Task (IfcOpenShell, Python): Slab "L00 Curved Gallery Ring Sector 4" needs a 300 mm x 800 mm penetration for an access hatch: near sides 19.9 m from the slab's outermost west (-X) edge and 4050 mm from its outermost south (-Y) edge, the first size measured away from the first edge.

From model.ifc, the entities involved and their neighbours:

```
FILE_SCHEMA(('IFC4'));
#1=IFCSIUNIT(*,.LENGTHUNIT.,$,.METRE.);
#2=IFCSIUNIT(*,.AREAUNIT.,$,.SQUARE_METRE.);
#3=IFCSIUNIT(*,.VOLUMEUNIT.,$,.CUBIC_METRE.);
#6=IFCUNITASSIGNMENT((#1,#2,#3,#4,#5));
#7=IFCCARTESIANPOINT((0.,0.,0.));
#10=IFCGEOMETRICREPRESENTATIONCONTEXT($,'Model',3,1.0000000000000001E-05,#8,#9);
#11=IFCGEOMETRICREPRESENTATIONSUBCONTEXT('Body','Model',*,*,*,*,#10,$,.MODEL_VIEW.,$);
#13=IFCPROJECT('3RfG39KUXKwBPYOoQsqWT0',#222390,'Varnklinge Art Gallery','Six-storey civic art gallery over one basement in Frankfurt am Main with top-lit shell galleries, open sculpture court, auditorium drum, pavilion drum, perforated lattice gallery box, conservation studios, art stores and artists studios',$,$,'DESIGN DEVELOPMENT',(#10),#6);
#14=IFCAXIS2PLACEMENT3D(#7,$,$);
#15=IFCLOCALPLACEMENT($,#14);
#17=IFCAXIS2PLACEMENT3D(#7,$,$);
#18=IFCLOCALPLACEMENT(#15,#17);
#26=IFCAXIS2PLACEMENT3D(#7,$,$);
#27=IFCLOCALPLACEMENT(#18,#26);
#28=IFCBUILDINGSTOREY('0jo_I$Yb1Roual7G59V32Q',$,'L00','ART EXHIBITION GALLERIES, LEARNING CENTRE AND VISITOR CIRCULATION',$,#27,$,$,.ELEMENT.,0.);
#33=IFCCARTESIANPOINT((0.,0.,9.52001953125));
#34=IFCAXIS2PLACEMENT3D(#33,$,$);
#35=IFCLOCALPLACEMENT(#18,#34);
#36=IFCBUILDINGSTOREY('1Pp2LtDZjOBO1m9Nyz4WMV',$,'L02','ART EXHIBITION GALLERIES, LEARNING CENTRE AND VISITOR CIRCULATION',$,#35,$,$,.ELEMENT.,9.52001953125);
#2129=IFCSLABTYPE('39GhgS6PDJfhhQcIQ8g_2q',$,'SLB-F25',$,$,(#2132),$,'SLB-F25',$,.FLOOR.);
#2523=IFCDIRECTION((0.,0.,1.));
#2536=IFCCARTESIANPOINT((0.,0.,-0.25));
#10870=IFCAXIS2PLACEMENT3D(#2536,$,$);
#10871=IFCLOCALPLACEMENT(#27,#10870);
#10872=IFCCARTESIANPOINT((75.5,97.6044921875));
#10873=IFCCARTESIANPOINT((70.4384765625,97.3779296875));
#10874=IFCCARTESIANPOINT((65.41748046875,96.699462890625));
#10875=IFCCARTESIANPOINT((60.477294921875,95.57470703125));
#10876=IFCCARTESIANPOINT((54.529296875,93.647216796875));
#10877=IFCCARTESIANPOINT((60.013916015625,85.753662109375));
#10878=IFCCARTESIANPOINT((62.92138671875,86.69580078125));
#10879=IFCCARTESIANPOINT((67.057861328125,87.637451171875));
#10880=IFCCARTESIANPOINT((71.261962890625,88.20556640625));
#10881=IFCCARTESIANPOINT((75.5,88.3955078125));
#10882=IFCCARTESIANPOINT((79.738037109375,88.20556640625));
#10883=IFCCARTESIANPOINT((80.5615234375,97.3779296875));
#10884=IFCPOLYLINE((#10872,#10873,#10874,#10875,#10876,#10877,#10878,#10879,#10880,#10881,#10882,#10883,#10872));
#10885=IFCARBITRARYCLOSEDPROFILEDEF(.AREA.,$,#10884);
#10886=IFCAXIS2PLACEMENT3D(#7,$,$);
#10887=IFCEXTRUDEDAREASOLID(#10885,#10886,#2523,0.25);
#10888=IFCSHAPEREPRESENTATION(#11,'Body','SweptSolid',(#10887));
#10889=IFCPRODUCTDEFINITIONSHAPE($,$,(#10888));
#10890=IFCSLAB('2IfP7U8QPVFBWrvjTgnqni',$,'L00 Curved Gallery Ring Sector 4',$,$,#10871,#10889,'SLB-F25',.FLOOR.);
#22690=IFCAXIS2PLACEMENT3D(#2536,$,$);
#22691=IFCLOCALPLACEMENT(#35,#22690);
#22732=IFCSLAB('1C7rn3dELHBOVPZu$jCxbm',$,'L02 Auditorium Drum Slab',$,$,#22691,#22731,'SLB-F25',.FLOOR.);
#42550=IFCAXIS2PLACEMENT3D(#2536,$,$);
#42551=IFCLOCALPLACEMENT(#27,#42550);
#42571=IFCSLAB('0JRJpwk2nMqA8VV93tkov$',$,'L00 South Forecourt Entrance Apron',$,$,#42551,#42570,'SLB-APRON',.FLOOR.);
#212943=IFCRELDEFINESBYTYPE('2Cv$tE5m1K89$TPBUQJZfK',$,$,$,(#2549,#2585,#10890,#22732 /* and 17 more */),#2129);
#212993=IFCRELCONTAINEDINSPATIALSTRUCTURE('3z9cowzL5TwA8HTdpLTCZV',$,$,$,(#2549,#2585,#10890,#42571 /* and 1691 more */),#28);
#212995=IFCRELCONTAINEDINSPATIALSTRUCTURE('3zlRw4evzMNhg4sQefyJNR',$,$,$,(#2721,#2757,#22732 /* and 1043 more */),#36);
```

```python
import numpy as np
import ifcopenshell
import ifcopenshell.api.feature
import ifcopenshell.api.geometry
import ifcopenshell.api.root
import ifcopenshell.geom
import ifcopenshell.util.placement
import ifcopenshell.util.representation
import ifcopenshell.util.shape
import ifcopenshell.util.unit

model = ifcopenshell.open("model.ifc")
unit_scale = ifcopenshell.util.unit.calculate_unit_scale(model)
settings = ifcopenshell.geom.settings()


def volume(element):
    """Net volume in cubic metres, openings subtracted."""
    shape = ifcopenshell.geom.create_shape(settings, element)
    return ifcopenshell.util.shape.get_volume(shape.geometry)


slab = model.by_guid("2IfP7U8QPVFBWrvjTgnqni")
before = volume(slab)

# Extent in the slab's own axes, in metres. The edges named are its -X and -Y sides.
slab_shape = ifcopenshell.geom.create_shape(settings, slab)
vertices = ifcopenshell.util.shape.get_vertices(slab_shape.geometry)
x_min, y_min, bottom = vertices.min(axis=0)
top = vertices[:, 2].max()

opening = ifcopenshell.api.root.create_entity(model, ifc_class="IfcOpeningElement", name="Access hatch opening", predefined_type="OPENING")
context = ifcopenshell.util.representation.get_context(model, "Model", "Body", "MODEL_VIEW")
width, depth = 0.3, 0.8
outline = [(0.0, 0.0), (width, 0.0), (width, depth), (0.0, depth), (0.0, 0.0)]
# Overshoot both faces by 50 mm so the cut is clean.
shape = ifcopenshell.api.geometry.add_slab_representation(
    model, context=context, depth=top - bottom + 0.1, polyline=outline
)
ifcopenshell.api.geometry.assign_representation(model, product=opening, representation=shape)

matrix = ifcopenshell.util.placement.get_local_placement(slab.ObjectPlacement)
matrix[:, 3] = matrix @ np.append(np.array([x_min + 19.9, y_min + 4.05, bottom - 0.05]) / unit_scale, 1.0)
ifcopenshell.api.geometry.edit_object_placement(model, product=opening, matrix=matrix, is_si=False)
ifcopenshell.api.feature.add_feature(model, feature=opening, element=slab)

after = volume(slab)

print(f"slab volume {before:.3f} -> {after:.3f} m3")

model.write("model_v2.ifc")
```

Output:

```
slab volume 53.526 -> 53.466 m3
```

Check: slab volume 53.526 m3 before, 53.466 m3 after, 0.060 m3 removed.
